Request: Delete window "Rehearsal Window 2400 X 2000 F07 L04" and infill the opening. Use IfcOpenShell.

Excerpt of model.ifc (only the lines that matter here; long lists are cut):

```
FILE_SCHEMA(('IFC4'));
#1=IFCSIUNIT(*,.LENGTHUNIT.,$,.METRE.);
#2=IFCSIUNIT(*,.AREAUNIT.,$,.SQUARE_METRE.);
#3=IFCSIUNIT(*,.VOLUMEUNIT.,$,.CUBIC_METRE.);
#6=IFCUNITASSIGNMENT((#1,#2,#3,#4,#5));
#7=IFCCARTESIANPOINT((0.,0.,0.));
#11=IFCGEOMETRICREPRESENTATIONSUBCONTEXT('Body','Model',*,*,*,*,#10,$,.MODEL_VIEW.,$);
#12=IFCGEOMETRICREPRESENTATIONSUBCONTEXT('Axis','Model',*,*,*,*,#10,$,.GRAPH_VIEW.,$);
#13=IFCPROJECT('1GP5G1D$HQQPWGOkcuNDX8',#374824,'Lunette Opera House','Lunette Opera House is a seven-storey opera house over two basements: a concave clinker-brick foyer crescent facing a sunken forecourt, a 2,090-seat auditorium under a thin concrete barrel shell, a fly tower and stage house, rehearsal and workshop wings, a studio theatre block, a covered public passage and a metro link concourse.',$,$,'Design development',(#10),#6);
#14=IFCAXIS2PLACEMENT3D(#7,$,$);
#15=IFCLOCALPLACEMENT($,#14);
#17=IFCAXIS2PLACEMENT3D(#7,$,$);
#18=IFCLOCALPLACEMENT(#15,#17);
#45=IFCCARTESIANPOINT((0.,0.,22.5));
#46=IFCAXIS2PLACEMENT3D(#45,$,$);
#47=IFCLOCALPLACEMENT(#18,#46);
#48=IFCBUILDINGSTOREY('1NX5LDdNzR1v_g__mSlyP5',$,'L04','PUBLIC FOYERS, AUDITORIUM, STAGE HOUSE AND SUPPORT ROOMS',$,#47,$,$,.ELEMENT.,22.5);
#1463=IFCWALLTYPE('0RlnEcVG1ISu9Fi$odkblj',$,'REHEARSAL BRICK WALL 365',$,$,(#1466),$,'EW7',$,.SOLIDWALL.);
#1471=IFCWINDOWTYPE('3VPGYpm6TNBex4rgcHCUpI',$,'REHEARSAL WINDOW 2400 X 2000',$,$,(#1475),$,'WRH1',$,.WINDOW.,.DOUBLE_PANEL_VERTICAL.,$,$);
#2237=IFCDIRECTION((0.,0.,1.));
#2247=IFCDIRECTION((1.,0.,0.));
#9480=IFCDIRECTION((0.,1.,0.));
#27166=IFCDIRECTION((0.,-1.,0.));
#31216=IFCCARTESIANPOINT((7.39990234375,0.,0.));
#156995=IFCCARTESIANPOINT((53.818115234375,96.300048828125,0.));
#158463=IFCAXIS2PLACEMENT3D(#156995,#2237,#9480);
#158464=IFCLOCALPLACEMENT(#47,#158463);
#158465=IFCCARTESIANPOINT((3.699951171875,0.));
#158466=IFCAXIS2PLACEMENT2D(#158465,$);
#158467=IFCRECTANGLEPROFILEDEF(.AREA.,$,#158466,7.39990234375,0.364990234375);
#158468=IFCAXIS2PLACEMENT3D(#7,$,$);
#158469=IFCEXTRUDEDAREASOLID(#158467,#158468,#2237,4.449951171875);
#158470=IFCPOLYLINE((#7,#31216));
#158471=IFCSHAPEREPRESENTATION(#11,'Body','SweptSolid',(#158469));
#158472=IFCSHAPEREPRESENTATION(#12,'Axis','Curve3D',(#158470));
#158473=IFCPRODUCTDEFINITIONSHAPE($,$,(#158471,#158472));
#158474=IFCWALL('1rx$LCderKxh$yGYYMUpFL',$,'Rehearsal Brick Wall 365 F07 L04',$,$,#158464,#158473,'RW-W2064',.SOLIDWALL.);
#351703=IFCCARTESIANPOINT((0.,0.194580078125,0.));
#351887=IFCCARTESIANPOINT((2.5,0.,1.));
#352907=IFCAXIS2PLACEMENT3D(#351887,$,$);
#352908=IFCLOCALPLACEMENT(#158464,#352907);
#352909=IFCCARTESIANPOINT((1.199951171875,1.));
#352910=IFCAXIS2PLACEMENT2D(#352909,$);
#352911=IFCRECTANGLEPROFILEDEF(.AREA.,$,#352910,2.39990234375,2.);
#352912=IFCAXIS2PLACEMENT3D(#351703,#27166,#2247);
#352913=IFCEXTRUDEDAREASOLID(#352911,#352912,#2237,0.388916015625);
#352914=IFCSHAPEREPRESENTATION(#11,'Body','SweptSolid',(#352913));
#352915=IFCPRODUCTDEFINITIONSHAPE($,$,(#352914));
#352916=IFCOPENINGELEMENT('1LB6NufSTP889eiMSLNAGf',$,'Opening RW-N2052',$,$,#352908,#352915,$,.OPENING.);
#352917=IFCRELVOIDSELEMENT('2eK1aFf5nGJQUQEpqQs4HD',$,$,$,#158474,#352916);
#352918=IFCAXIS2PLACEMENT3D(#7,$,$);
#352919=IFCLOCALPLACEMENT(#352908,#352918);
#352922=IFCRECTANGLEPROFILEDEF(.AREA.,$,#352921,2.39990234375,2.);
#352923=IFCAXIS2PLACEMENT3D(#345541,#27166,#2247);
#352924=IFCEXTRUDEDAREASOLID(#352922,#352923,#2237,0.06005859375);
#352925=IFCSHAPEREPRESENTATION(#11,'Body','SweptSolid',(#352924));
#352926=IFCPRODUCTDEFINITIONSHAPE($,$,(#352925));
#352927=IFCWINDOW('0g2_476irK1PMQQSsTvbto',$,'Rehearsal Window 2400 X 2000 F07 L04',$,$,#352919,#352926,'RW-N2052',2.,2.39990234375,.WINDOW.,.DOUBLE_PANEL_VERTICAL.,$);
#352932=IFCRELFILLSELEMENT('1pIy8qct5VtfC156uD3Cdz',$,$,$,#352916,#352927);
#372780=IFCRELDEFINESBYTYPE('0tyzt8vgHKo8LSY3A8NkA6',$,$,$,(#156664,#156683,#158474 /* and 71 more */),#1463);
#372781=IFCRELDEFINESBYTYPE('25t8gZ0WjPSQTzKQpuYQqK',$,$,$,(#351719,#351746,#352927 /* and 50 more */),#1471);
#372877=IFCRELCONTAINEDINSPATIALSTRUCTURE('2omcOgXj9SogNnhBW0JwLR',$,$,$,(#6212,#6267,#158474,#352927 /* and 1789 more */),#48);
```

```python
import ifcopenshell
import ifcopenshell.api.feature
import ifcopenshell.api.root
import ifcopenshell.geom
import ifcopenshell.util.shape

model = ifcopenshell.open("model.ifc")
settings = ifcopenshell.geom.settings()


def volume(element):
    """Net volume in cubic metres, openings subtracted."""
    shape = ifcopenshell.geom.create_shape(settings, element)
    return ifcopenshell.util.shape.get_volume(shape.geometry)


window = model.by_guid("0g2_476irK1PMQQSsTvbto")
opening = window.FillsVoids[0].RelatingOpeningElement
wall = opening.VoidsElements[0].RelatingBuildingElement
before = volume(wall)

ifcopenshell.api.root.remove_product(model, product=window)
ifcopenshell.api.feature.remove_feature(model, feature=opening)

after = volume(wall)

print(f"wall volume {before:.3f} -> {after:.3f} m3")

model.write("model_rev.ifc")
```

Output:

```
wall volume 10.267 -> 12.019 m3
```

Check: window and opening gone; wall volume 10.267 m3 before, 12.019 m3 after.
